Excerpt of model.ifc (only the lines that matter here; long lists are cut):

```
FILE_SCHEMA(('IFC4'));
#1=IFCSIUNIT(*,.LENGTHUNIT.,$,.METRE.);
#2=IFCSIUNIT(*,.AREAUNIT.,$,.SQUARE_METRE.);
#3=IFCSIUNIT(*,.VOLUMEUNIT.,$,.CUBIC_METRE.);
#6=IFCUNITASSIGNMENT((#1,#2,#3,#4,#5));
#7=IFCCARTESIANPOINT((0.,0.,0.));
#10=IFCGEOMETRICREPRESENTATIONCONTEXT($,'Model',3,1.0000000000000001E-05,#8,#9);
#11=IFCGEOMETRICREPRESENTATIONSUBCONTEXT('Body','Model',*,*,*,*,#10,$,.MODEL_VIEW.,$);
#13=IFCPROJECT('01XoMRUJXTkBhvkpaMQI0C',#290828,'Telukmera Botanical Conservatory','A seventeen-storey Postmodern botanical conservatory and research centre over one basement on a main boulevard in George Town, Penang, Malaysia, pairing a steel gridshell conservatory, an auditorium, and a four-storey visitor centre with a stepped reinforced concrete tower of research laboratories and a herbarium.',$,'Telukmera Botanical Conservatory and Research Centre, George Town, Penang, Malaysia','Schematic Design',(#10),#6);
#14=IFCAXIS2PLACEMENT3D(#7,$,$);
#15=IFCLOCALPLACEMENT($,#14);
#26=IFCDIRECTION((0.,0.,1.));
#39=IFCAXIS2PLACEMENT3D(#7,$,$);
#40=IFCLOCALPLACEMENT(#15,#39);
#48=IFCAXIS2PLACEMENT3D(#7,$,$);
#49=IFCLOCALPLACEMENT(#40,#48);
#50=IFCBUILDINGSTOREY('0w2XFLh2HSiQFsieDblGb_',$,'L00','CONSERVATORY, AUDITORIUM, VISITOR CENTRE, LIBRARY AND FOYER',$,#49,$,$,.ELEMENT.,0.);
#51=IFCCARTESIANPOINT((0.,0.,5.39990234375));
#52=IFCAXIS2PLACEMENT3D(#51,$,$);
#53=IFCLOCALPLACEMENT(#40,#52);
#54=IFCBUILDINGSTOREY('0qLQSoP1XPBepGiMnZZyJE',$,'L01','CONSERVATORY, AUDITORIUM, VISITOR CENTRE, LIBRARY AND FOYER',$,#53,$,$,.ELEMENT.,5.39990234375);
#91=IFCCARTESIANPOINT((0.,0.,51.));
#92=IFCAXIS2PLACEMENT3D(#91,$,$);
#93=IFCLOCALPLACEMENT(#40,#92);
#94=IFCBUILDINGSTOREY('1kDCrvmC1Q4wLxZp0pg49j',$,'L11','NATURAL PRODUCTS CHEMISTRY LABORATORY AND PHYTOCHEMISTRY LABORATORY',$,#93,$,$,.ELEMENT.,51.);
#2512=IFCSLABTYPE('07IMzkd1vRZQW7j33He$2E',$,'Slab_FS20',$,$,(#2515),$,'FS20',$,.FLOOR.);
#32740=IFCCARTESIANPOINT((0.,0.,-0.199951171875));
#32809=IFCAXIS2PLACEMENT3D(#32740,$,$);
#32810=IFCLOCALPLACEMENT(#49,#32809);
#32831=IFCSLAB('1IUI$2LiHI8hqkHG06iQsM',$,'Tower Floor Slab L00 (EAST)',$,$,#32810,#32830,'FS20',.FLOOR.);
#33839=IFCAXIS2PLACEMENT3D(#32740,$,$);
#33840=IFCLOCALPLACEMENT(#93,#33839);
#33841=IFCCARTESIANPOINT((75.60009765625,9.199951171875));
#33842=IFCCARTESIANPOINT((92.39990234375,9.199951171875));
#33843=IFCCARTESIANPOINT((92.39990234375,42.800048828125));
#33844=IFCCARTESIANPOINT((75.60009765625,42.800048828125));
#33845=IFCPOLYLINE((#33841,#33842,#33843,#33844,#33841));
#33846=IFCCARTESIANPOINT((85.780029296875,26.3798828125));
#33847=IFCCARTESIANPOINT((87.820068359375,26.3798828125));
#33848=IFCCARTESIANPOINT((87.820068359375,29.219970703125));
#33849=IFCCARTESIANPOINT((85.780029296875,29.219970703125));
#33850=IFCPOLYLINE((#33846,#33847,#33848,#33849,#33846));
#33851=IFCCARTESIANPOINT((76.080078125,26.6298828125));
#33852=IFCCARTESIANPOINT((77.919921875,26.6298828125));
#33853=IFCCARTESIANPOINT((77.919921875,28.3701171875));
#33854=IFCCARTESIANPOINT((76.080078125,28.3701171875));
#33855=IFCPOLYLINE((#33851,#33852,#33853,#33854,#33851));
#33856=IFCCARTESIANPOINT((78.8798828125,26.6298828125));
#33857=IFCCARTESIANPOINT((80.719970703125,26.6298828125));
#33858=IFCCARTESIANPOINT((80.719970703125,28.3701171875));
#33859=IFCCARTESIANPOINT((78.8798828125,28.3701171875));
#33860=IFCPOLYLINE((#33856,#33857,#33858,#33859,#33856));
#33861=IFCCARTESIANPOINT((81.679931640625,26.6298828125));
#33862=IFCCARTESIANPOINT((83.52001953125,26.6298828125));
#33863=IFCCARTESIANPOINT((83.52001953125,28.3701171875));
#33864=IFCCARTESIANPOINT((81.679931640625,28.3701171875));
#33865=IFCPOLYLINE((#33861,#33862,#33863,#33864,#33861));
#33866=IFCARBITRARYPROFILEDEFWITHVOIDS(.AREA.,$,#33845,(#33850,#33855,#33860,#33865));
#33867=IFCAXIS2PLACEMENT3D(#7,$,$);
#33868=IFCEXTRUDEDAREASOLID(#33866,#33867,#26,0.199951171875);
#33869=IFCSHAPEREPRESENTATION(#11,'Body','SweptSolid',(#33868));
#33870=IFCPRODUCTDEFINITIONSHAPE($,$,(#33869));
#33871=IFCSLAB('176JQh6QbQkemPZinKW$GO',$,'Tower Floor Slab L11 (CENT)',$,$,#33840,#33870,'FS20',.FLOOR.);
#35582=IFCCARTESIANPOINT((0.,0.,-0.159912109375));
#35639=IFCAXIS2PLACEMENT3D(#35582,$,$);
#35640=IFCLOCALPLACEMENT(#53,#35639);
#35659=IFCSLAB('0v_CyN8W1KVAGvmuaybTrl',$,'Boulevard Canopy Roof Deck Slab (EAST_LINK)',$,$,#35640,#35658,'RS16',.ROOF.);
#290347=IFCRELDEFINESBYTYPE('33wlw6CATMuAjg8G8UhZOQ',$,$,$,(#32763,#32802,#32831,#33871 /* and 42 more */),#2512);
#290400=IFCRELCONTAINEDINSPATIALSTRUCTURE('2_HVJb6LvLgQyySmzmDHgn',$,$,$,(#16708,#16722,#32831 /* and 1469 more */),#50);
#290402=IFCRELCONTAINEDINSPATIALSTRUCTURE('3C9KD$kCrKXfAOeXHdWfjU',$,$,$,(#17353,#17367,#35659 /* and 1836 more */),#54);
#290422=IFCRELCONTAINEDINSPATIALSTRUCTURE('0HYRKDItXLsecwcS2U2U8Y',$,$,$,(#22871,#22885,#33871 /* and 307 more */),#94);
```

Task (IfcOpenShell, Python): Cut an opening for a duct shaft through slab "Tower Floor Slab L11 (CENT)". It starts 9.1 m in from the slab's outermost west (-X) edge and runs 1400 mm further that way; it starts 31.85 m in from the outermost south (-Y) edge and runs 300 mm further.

```python
import numpy as np
import ifcopenshell
import ifcopenshell.api.feature
import ifcopenshell.api.geometry
import ifcopenshell.api.root
import ifcopenshell.geom
import ifcopenshell.util.placement
import ifcopenshell.util.representation
import ifcopenshell.util.shape
import ifcopenshell.util.unit

model = ifcopenshell.open("model.ifc")
unit_scale = ifcopenshell.util.unit.calculate_unit_scale(model)
settings = ifcopenshell.geom.settings()


def volume(element):
    """Net volume in cubic metres, openings subtracted."""
    shape = ifcopenshell.geom.create_shape(settings, element)
    return ifcopenshell.util.shape.get_volume(shape.geometry)


slab = model.by_id(33871)
before = volume(slab)

# Extent in the slab's own axes, in metres. The edges named are its -X and -Y sides.
slab_shape = ifcopenshell.geom.create_shape(settings, slab)
vertices = ifcopenshell.util.shape.get_vertices(slab_shape.geometry)
x_min, y_min, bottom = vertices.min(axis=0)
top = vertices[:, 2].max()

opening = ifcopenshell.api.root.create_entity(model, ifc_class="IfcOpeningElement", name="Duct shaft opening", predefined_type="OPENING")
context = ifcopenshell.util.representation.get_context(model, "Model", "Body", "MODEL_VIEW")
width, depth = 1.4, 0.3
outline = [(0.0, 0.0), (width, 0.0), (width, depth), (0.0, depth), (0.0, 0.0)]
# Overshoot both faces by 50 mm so the cut is clean.
shape = ifcopenshell.api.geometry.add_slab_representation(
    model, context=context, depth=top - bottom + 0.1, polyline=outline
)
ifcopenshell.api.geometry.assign_representation(model, product=opening, representation=shape)

matrix = ifcopenshell.util.placement.get_local_placement(slab.ObjectPlacement)
matrix[:, 3] = matrix @ np.append(np.array([x_min + 9.1, y_min + 31.85, bottom - 0.05]) / unit_scale, 1.0)
ifcopenshell.api.geometry.edit_object_placement(model, product=opening, matrix=matrix, is_si=False)
ifcopenshell.api.feature.add_feature(model, feature=opening, element=slab)

after = volume(slab)

print(f"slab volume {before:.3f} -> {after:.3f} m3")

model.write("model_updated.ifc")
```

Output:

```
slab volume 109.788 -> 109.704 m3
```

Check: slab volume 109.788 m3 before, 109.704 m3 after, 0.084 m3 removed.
